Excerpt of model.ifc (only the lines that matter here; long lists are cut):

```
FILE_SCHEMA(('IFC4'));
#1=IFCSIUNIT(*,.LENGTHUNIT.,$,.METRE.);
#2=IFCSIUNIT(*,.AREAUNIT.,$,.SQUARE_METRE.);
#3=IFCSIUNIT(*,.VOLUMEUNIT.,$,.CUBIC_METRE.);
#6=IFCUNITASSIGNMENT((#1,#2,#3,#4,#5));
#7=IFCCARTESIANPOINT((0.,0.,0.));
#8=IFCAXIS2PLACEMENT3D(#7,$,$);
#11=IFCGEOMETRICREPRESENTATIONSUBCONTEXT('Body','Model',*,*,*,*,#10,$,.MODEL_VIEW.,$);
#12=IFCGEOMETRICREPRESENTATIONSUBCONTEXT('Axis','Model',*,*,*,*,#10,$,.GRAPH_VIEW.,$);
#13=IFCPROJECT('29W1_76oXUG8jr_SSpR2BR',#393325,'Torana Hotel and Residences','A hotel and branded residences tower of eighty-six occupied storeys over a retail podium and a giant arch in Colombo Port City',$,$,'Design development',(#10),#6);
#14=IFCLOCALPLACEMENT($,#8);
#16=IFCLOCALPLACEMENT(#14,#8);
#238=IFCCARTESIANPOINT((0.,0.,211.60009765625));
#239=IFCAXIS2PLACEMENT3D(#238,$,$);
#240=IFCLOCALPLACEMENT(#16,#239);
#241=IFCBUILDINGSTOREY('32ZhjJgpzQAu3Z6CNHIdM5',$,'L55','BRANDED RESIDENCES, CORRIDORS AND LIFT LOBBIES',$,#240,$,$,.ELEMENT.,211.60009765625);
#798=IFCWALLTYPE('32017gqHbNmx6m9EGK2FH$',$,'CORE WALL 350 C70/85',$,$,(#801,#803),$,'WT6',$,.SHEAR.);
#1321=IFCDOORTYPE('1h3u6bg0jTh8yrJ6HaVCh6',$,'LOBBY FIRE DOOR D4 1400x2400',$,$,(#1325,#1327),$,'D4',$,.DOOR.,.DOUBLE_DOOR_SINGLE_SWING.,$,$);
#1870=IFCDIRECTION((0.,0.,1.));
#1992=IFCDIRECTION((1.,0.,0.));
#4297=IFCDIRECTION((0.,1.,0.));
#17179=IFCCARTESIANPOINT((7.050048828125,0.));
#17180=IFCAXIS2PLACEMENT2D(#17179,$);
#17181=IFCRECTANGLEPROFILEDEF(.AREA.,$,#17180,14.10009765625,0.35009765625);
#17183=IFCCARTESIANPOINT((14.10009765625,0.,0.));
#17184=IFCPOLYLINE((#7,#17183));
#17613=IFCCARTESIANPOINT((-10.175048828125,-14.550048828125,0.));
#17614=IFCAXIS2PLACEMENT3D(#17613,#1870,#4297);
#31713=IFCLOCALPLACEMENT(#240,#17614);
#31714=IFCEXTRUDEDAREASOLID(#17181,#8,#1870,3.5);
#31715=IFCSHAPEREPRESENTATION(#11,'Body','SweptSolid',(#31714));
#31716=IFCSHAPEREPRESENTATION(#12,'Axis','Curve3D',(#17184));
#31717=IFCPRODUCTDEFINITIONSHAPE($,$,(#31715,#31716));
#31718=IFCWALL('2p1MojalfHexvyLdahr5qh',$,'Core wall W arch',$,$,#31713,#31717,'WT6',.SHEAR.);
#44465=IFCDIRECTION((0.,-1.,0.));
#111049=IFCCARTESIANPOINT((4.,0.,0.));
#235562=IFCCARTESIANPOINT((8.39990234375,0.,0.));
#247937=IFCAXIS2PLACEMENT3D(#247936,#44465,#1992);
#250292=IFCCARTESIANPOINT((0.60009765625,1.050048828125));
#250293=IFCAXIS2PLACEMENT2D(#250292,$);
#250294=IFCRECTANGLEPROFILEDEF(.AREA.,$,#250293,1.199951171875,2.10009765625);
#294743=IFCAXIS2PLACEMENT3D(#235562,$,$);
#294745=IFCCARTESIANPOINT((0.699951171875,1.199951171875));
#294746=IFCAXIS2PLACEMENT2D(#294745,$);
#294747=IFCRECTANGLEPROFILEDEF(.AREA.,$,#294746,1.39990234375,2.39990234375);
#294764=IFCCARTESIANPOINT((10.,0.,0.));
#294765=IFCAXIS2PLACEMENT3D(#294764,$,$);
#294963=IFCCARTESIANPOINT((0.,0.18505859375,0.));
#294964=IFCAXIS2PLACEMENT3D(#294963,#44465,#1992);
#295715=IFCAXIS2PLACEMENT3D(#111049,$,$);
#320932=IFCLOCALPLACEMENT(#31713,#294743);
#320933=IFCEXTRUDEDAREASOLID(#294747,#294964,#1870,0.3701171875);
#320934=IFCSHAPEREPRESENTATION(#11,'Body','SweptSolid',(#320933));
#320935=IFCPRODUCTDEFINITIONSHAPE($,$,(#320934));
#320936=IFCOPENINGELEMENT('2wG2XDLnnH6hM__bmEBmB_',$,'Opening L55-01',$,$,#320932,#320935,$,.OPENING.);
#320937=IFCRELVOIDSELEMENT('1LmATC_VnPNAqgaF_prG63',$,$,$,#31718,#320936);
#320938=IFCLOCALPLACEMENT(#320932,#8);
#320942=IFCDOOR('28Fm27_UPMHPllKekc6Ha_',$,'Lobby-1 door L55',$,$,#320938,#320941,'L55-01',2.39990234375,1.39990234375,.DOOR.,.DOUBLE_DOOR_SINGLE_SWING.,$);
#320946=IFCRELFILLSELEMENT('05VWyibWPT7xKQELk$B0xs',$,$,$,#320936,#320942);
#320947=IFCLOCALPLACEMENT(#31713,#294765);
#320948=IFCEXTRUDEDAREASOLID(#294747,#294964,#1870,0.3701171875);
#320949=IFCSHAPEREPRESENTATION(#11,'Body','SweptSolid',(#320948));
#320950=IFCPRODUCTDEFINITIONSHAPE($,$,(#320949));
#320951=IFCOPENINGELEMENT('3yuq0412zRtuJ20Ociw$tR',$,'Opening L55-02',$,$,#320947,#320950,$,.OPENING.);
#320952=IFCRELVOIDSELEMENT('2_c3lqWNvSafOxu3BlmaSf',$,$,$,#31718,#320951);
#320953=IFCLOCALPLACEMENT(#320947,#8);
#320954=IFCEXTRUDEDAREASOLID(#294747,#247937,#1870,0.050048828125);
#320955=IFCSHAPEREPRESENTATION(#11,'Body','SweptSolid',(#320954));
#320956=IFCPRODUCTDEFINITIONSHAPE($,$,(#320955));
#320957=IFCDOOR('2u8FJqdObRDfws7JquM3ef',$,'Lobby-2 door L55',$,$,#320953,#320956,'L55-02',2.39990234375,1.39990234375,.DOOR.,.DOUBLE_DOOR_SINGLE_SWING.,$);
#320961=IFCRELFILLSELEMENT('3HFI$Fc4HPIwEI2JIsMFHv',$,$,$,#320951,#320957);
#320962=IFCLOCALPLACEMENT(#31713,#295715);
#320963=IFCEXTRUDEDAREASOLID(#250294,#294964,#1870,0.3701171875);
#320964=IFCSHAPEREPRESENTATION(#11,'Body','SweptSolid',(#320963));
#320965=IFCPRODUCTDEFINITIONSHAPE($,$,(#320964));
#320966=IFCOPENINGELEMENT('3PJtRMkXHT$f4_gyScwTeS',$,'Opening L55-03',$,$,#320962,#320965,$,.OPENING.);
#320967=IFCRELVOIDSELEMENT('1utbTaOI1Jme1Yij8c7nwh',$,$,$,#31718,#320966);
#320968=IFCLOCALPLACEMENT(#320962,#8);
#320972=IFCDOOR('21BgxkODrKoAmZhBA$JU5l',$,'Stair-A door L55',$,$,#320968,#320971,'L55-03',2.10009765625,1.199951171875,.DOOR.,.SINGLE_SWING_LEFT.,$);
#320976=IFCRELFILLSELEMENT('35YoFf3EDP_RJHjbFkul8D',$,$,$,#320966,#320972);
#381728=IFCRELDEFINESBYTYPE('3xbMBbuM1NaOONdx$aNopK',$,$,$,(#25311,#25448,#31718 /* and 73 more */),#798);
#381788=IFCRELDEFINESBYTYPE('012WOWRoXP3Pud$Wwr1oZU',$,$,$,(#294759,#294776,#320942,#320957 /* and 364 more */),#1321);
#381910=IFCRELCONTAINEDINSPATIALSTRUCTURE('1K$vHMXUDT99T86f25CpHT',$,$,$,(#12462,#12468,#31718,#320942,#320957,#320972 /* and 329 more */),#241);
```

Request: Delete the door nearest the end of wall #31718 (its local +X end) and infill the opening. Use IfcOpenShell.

```python
import ifcopenshell
import ifcopenshell.api.feature
import ifcopenshell.api.root
import ifcopenshell.geom
import ifcopenshell.util.shape

model = ifcopenshell.open("model.ifc")
settings = ifcopenshell.geom.settings()


def volume(element):
    """Net volume in cubic metres, openings subtracted."""
    shape = ifcopenshell.geom.create_shape(settings, element)
    return ifcopenshell.util.shape.get_volume(shape.geometry)


door = model.by_guid("2u8FJqdObRDfws7JquM3ef")
opening = door.FillsVoids[0].RelatingOpeningElement
wall = opening.VoidsElements[0].RelatingBuildingElement
before = volume(wall)

ifcopenshell.api.root.remove_product(model, product=door)
ifcopenshell.api.feature.remove_feature(model, feature=opening)

after = volume(wall)

print(f"wall volume {before:.3f} -> {after:.3f} m3")

model.write("model_v2.ifc")
```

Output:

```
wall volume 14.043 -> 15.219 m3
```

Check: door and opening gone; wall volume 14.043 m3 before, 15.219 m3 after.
